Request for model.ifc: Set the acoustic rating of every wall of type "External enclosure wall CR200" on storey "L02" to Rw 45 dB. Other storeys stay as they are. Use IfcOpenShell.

First a look at what the model holds.

```python
import ifcopenshell
import ifcopenshell.util.element

model = ifcopenshell.open("model.ifc")
print(model.schema)
storey = next(s for s in model.by_type("IfcBuildingStorey") if s.Name == "L02")
walls = [e for e in ifcopenshell.util.element.get_decomposition(storey) if e.is_a("IfcWall")]
seen = {}
for e in walls:
    element_type = ifcopenshell.util.element.get_type(e)
    key = (element_type.Name if element_type != e and element_type else None, ifcopenshell.util.element.get_pset(e, "Pset_WallCommon", "AcousticRating"))
    seen[key] = seen.get(key, 0) + 1
for (name, value), count in sorted(seen.items(), key=str):
    print(count, "x", name, "|", value)
```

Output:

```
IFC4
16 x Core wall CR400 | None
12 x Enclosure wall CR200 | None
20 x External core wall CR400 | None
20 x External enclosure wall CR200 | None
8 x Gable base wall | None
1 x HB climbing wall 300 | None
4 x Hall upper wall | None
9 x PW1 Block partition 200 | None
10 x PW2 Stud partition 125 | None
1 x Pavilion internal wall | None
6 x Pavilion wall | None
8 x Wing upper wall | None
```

```python
import ifcopenshell
import ifcopenshell.api.pset
import ifcopenshell.util.element

model = ifcopenshell.open("model.ifc")

storey = next(s for s in model.by_type("IfcBuildingStorey") if s.Name == "L02")
walls = [e for e in ifcopenshell.util.element.get_decomposition(storey) if e.is_a("IfcWall")]

count = 0
for e in walls:
    element_type = ifcopenshell.util.element.get_type(e)
    if element_type in (None, e) or element_type.Name != "External enclosure wall CR200":
        continue
    # add_pset returns the element's existing set when there is one.
    pset = ifcopenshell.api.pset.add_pset(model, product=e, name="Pset_WallCommon")
    ifcopenshell.api.pset.edit_pset(model, pset=pset, properties={"AcousticRating": "Rw 45 dB"})
    count += 1

print(count, "walls updated")

model.write("model_rev.ifc")
```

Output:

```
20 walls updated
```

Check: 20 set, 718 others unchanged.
